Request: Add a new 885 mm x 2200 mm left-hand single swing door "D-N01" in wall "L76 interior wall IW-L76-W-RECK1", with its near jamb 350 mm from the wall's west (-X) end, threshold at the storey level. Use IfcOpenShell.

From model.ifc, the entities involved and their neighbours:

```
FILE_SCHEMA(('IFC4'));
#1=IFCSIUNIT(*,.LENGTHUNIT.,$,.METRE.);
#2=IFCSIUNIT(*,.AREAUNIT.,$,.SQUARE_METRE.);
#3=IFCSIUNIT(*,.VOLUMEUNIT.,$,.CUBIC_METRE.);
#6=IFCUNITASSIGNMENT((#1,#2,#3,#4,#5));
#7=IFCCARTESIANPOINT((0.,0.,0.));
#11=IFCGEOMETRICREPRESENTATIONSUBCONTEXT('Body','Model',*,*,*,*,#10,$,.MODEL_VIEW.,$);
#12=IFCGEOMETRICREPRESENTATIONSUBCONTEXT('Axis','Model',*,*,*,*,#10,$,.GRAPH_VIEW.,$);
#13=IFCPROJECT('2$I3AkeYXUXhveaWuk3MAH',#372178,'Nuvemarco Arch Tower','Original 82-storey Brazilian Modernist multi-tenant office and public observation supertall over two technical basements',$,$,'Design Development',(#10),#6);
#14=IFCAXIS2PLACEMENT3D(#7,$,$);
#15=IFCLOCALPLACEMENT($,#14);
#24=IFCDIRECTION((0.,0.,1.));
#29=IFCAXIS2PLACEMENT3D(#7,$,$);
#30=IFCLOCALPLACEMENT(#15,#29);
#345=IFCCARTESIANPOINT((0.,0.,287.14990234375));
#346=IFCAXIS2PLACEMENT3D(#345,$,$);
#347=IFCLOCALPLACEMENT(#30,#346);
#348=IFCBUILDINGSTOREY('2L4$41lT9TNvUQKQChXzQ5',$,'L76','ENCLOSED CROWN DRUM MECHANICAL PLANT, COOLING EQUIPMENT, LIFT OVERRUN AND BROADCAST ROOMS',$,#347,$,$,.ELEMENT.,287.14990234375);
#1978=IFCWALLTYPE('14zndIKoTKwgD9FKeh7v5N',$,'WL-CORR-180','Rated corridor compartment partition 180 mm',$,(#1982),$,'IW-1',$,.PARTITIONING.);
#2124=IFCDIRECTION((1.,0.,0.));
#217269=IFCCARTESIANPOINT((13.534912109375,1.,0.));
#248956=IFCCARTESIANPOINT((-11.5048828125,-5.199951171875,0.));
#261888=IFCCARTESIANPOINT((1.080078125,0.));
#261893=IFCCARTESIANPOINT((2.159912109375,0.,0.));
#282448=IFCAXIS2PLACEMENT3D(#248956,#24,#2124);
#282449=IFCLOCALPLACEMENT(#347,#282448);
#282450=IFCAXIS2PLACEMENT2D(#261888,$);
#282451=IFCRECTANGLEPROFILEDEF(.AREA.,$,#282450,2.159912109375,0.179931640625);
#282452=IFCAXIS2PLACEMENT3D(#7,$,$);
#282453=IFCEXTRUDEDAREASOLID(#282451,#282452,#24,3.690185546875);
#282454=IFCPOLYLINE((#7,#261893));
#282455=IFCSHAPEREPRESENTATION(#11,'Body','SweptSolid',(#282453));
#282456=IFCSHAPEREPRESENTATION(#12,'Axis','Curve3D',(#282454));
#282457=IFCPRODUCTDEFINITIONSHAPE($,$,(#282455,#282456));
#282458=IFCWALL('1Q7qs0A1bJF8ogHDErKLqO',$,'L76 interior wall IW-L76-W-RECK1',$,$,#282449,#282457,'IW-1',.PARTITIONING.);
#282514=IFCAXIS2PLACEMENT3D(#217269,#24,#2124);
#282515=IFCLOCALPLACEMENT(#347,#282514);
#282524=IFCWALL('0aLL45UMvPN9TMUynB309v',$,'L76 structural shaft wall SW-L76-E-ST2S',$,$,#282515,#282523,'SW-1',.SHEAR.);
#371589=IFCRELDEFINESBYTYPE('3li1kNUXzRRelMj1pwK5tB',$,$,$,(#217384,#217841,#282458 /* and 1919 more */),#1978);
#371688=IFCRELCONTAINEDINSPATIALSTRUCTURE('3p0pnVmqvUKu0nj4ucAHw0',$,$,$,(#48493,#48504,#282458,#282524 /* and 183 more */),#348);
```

```python
import numpy as np
import ifcopenshell
import ifcopenshell.api.feature
import ifcopenshell.api.geometry
import ifcopenshell.api.root
import ifcopenshell.api.spatial
import ifcopenshell.geom
import ifcopenshell.util.element
import ifcopenshell.util.placement
import ifcopenshell.util.representation
import ifcopenshell.util.shape
import ifcopenshell.util.unit

model = ifcopenshell.open("model.ifc")
unit_scale = ifcopenshell.util.unit.calculate_unit_scale(model)
settings = ifcopenshell.geom.settings()


def volume(element):
    """Net volume in cubic metres, openings subtracted."""
    shape = ifcopenshell.geom.create_shape(settings, element)
    return ifcopenshell.util.shape.get_volume(shape.geometry)


wall = model.by_id(282458)
storey = ifcopenshell.util.element.get_container(wall, ifc_class="IfcBuildingStorey")
context = ifcopenshell.util.representation.get_context(model, "Model", "Body", "MODEL_VIEW")
before = volume(wall)

width, height, from_end, sill = 0.885, 2.2, 0.35, 0.0  # metres

# The wall runs along its own X axis, and the end named is its -X end.
wall_shape = ifcopenshell.geom.create_shape(settings, wall)
x, y, z = ifcopenshell.util.shape.get_vertices(wall_shape.geometry).T
start = x.min() + from_end
face, thickness = float(y.min()), float(y.max() - y.min())
wall_matrix = ifcopenshell.util.placement.get_local_placement(wall.ObjectPlacement)
level = ifcopenshell.util.placement.get_local_placement(storey.ObjectPlacement)[2, 3]


def in_wall(x, y):
    """Placement at x, y metres in the wall's axes, at sill height."""
    matrix = wall_matrix.copy()
    matrix[:, 3] = wall_matrix @ np.array([x / unit_scale, y / unit_scale, 0.0, 1.0])
    matrix[2, 3] = level + sill / unit_scale
    return matrix


# Opening: a box that overshoots both wall faces by 50 mm.
opening = ifcopenshell.api.root.create_entity(model, ifc_class="IfcOpeningElement", predefined_type="OPENING")
box = ifcopenshell.api.geometry.add_wall_representation(
    model, context=context, length=width, height=height, thickness=thickness + 0.1
)
ifcopenshell.api.geometry.assign_representation(model, product=opening, representation=box)
ifcopenshell.api.geometry.edit_object_placement(model, product=opening, matrix=in_wall(start, face - 0.05), is_si=False)
ifcopenshell.api.feature.add_feature(model, feature=opening, element=wall)

door = ifcopenshell.api.root.create_entity(model, ifc_class="IfcDoor", name="D-N01", predefined_type="DOOR")
door.OverallWidth, door.OverallHeight = width / unit_scale, height / unit_scale
door.OperationType = "SINGLE_SWING_LEFT"
body = ifcopenshell.api.geometry.add_door_representation(
    model,
    context=context,
    overall_width=door.OverallWidth,
    overall_height=door.OverallHeight,
    operation_type="SINGLE_SWING_LEFT",
    lining_properties={"LiningDepth": thickness / unit_scale, "ThresholdDepth": thickness / unit_scale},
)
ifcopenshell.api.geometry.assign_representation(model, product=door, representation=body)
ifcopenshell.api.spatial.assign_container(model, products=[door], relating_structure=storey)
ifcopenshell.api.feature.add_filling(model, opening=opening, element=door)

# The lining spans the wall, so the door starts at the wall face.
ifcopenshell.api.geometry.edit_object_placement(model, product=door, matrix=in_wall(start, face), is_si=False)

after = volume(wall)

print(f"wall volume {before:.3f} -> {after:.3f} m3")

model.write("model_updated.ifc")
```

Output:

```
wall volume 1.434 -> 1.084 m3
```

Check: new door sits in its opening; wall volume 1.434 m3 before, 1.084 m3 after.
